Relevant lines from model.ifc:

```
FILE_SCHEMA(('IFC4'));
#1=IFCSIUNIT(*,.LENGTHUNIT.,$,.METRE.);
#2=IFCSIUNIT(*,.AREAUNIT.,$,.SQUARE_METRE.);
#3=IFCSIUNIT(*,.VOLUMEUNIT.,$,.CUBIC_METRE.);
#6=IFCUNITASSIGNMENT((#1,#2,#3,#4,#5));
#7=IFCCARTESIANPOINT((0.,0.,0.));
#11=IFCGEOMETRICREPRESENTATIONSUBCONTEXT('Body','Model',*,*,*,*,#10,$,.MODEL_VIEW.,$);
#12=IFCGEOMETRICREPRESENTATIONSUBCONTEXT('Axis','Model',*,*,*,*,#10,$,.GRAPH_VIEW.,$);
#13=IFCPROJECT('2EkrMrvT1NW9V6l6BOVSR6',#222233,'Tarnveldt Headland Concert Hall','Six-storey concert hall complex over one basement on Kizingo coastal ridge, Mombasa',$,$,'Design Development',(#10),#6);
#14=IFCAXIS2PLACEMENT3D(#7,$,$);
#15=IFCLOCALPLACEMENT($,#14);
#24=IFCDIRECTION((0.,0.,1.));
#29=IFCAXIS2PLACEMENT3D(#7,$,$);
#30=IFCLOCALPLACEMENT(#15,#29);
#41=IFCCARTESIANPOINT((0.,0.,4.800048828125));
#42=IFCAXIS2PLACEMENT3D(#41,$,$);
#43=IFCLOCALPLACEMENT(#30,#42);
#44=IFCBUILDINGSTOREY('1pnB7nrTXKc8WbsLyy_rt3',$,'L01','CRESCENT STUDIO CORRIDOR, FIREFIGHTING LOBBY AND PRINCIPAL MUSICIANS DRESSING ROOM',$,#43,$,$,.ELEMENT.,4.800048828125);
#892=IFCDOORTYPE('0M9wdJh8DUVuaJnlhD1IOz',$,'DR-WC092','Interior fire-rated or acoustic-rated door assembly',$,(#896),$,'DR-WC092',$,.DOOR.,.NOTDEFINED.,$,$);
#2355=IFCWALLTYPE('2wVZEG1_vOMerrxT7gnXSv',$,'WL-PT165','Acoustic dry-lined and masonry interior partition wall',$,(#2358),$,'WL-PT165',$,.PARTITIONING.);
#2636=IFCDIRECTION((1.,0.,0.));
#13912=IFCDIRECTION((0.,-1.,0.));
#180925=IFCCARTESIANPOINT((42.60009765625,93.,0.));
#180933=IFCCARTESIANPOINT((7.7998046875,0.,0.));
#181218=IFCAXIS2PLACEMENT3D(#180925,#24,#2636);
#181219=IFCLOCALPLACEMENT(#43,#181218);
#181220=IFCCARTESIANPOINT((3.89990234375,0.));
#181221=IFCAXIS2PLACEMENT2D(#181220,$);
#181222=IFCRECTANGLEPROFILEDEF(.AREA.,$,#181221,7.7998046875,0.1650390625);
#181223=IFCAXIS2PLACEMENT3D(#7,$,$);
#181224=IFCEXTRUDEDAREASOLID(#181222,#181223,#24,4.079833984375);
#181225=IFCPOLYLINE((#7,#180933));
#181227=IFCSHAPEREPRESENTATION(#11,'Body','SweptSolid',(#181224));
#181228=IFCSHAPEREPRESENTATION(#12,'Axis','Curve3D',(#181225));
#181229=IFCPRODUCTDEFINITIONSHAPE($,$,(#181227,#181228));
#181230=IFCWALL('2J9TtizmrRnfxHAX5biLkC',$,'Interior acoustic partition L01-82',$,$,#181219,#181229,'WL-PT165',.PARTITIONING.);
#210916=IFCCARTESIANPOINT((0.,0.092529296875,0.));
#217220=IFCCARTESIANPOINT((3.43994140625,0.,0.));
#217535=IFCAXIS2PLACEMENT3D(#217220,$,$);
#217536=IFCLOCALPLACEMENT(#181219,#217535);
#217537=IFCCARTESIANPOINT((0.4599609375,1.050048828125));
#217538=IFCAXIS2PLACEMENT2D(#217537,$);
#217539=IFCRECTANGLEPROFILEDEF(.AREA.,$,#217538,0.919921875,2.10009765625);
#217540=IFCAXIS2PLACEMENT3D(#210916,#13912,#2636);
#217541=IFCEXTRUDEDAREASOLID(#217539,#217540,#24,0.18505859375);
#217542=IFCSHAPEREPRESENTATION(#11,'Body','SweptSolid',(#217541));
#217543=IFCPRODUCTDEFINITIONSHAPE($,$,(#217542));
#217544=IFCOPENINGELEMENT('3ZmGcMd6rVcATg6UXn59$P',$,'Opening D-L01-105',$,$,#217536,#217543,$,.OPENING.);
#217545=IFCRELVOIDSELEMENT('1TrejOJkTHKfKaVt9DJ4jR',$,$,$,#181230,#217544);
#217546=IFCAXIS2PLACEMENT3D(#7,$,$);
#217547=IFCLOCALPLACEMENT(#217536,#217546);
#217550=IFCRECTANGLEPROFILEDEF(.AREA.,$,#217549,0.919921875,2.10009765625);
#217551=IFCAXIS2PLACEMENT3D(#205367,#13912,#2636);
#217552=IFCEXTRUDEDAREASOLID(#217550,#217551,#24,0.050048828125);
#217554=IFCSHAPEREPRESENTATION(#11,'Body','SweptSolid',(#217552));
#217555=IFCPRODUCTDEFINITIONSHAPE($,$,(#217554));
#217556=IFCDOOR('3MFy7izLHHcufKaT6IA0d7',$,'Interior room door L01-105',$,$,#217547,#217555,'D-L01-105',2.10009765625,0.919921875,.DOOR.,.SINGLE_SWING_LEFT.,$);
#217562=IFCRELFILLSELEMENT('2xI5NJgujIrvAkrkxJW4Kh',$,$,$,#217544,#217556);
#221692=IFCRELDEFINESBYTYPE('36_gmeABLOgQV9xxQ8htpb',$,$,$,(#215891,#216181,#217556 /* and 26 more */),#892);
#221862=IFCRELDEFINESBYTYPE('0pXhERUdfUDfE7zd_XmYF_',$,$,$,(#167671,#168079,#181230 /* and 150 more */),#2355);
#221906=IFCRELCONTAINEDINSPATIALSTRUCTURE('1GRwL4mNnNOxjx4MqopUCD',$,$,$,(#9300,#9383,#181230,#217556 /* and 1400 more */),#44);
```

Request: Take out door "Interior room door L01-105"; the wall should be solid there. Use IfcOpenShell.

```python
import ifcopenshell
import ifcopenshell.api.feature
import ifcopenshell.api.root
import ifcopenshell.geom
import ifcopenshell.util.shape

model = ifcopenshell.open("model.ifc")
settings = ifcopenshell.geom.settings()


def volume(element):
    """Net volume in cubic metres, openings subtracted."""
    shape = ifcopenshell.geom.create_shape(settings, element)
    return ifcopenshell.util.shape.get_volume(shape.geometry)


door = model.by_guid("3MFy7izLHHcufKaT6IA0d7")
opening = door.FillsVoids[0].RelatingOpeningElement
wall = opening.VoidsElements[0].RelatingBuildingElement
before = volume(wall)

ifcopenshell.api.root.remove_product(model, product=door)
ifcopenshell.api.feature.remove_feature(model, feature=opening)

after = volume(wall)

print(f"wall volume {before:.3f} -> {after:.3f} m3")

model.write("model_edited.ifc")
```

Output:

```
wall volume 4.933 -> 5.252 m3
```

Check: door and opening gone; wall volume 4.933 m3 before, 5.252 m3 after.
